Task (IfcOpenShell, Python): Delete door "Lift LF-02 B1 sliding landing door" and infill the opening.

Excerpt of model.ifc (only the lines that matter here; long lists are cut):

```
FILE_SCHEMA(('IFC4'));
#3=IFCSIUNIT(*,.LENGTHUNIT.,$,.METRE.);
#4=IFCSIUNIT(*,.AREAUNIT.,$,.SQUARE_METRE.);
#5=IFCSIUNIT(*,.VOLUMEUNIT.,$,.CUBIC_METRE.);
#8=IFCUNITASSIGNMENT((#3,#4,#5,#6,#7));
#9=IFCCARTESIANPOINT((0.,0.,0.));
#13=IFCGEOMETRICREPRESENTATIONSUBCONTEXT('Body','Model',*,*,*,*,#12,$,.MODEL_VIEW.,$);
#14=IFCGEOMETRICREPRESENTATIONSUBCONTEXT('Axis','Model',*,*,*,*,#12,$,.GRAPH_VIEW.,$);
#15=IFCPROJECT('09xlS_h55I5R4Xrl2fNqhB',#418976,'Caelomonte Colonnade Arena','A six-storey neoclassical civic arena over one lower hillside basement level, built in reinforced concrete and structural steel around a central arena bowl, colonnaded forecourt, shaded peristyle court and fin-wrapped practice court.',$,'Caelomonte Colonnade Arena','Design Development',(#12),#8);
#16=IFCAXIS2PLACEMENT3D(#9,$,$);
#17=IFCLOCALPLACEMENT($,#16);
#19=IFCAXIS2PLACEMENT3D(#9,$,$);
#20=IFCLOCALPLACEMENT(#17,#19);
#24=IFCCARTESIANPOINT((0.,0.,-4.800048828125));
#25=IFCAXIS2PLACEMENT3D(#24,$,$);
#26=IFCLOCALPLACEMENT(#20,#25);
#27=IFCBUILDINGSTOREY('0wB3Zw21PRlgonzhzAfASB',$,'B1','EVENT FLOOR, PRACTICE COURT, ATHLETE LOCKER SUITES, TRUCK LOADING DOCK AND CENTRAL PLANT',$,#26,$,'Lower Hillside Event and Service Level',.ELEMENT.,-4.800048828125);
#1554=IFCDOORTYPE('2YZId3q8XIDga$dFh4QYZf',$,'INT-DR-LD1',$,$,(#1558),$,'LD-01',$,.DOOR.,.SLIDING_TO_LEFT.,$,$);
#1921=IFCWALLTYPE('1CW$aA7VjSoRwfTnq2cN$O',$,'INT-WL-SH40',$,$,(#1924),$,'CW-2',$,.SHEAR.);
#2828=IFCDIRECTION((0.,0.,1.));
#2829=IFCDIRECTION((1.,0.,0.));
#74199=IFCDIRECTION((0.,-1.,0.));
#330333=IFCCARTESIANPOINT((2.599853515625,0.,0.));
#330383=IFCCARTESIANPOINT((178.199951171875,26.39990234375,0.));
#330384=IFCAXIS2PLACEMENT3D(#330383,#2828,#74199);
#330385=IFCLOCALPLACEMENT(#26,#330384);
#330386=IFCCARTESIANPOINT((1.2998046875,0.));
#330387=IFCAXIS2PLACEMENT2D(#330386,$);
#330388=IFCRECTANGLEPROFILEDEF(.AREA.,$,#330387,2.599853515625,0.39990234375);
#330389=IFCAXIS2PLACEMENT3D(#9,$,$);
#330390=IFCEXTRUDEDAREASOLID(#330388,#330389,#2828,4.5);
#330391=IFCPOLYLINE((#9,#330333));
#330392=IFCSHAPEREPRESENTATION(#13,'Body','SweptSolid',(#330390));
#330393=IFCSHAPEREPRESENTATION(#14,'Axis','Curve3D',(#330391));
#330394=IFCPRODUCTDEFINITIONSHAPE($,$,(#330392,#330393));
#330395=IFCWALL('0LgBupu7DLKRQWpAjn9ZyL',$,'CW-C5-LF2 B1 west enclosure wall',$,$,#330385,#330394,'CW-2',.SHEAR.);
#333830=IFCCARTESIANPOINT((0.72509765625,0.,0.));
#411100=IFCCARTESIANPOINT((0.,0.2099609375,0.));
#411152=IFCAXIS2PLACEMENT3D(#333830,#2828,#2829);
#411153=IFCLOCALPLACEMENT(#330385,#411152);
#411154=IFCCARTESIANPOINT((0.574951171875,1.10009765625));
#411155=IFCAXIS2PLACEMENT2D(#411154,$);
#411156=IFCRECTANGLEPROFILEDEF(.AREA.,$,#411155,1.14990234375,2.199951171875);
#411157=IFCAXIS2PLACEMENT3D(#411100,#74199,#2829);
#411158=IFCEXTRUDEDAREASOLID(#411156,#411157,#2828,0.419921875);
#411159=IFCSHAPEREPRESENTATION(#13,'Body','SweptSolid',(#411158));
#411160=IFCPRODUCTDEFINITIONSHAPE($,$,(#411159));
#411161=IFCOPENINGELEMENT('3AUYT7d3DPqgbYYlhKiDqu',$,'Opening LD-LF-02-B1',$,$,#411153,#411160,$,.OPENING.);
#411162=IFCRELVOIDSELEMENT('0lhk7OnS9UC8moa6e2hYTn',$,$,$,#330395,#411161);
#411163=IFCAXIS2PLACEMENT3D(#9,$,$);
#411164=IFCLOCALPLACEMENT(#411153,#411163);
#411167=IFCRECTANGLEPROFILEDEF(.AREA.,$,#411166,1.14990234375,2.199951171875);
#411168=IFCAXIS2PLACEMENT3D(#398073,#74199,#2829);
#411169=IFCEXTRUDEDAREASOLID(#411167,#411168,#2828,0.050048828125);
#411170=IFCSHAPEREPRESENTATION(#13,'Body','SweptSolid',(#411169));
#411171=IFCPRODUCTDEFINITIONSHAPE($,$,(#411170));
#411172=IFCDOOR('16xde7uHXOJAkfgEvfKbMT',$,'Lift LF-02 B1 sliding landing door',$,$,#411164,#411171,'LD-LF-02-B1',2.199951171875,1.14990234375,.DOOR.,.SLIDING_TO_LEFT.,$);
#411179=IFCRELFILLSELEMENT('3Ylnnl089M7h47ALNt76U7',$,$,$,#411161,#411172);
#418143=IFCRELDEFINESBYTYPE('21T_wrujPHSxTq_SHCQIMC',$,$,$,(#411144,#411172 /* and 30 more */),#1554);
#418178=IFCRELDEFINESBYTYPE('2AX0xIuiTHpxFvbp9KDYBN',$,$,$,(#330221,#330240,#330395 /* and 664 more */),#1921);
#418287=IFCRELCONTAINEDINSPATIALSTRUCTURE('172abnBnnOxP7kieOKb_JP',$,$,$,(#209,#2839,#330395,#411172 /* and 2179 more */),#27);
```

```python
import ifcopenshell
import ifcopenshell.api.feature
import ifcopenshell.api.root
import ifcopenshell.geom
import ifcopenshell.util.shape

model = ifcopenshell.open("model.ifc")
settings = ifcopenshell.geom.settings()


def volume(element):
    """Net volume in cubic metres, openings subtracted."""
    shape = ifcopenshell.geom.create_shape(settings, element)
    return ifcopenshell.util.shape.get_volume(shape.geometry)


door = model.by_id(411172)
opening = door.FillsVoids[0].RelatingOpeningElement
wall = opening.VoidsElements[0].RelatingBuildingElement
before = volume(wall)

ifcopenshell.api.root.remove_product(model, product=door)
ifcopenshell.api.feature.remove_feature(model, feature=opening)

after = volume(wall)

print(f"wall volume {before:.3f} -> {after:.3f} m3")

model.write("model_v2.ifc")
```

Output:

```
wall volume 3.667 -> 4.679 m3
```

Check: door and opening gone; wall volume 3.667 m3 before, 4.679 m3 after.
